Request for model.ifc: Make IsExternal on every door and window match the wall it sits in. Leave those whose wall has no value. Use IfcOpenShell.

First a look at what the model holds.

```python
import ifcopenshell
import ifcopenshell.util.element

model = ifcopenshell.open("model.ifc")
print(model.schema)
seen = {}
for e in model.by_type("IfcDoor") + model.by_type("IfcWindow"):
    if not e.FillsVoids:
        continue
    host = e.FillsVoids[0].RelatingOpeningElement.VoidsElements[0].RelatingBuildingElement
    own = ifcopenshell.util.element.get_pset(e, f"Pset_{e.is_a()[3:].removesuffix('StandardCase')}Common", "IsExternal")
    wall = ifcopenshell.util.element.get_pset(host, "Pset_WallCommon", "IsExternal")
    seen[e.is_a(), own, wall] = seen.get((e.is_a(), own, wall), 0) + 1
for (cls, own, wall), count in sorted(seen.items(), key=str):
    print(count, cls, "IsExternal:", own, "| host wall:", wall)
```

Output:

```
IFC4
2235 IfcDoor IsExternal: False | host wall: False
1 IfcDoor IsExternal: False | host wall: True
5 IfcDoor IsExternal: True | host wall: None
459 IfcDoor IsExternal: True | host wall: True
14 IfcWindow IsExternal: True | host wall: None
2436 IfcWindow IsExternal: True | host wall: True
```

```python
import ifcopenshell
import ifcopenshell.api.pset
import ifcopenshell.util.element

model = ifcopenshell.open("model.ifc")

count = 0
for ifc_class, pset_name in (("IfcDoor", "Pset_DoorCommon"), ("IfcWindow", "Pset_WindowCommon")):
    for e in model.by_type(ifc_class):
        if not e.FillsVoids:
            continue
        host = e.FillsVoids[0].RelatingOpeningElement.VoidsElements[0].RelatingBuildingElement
        external = ifcopenshell.util.element.get_pset(host, "Pset_WallCommon", "IsExternal")
        if external is None or ifcopenshell.util.element.get_pset(e, pset_name, "IsExternal") == external:
            continue
        pset = ifcopenshell.api.pset.add_pset(model, product=e, name=pset_name)
        ifcopenshell.api.pset.edit_pset(model, pset=pset, properties={"IsExternal": external})
        count += 1

print(count, "updated")

model.write("model-out.ifc")
```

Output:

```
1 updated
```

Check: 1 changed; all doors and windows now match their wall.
